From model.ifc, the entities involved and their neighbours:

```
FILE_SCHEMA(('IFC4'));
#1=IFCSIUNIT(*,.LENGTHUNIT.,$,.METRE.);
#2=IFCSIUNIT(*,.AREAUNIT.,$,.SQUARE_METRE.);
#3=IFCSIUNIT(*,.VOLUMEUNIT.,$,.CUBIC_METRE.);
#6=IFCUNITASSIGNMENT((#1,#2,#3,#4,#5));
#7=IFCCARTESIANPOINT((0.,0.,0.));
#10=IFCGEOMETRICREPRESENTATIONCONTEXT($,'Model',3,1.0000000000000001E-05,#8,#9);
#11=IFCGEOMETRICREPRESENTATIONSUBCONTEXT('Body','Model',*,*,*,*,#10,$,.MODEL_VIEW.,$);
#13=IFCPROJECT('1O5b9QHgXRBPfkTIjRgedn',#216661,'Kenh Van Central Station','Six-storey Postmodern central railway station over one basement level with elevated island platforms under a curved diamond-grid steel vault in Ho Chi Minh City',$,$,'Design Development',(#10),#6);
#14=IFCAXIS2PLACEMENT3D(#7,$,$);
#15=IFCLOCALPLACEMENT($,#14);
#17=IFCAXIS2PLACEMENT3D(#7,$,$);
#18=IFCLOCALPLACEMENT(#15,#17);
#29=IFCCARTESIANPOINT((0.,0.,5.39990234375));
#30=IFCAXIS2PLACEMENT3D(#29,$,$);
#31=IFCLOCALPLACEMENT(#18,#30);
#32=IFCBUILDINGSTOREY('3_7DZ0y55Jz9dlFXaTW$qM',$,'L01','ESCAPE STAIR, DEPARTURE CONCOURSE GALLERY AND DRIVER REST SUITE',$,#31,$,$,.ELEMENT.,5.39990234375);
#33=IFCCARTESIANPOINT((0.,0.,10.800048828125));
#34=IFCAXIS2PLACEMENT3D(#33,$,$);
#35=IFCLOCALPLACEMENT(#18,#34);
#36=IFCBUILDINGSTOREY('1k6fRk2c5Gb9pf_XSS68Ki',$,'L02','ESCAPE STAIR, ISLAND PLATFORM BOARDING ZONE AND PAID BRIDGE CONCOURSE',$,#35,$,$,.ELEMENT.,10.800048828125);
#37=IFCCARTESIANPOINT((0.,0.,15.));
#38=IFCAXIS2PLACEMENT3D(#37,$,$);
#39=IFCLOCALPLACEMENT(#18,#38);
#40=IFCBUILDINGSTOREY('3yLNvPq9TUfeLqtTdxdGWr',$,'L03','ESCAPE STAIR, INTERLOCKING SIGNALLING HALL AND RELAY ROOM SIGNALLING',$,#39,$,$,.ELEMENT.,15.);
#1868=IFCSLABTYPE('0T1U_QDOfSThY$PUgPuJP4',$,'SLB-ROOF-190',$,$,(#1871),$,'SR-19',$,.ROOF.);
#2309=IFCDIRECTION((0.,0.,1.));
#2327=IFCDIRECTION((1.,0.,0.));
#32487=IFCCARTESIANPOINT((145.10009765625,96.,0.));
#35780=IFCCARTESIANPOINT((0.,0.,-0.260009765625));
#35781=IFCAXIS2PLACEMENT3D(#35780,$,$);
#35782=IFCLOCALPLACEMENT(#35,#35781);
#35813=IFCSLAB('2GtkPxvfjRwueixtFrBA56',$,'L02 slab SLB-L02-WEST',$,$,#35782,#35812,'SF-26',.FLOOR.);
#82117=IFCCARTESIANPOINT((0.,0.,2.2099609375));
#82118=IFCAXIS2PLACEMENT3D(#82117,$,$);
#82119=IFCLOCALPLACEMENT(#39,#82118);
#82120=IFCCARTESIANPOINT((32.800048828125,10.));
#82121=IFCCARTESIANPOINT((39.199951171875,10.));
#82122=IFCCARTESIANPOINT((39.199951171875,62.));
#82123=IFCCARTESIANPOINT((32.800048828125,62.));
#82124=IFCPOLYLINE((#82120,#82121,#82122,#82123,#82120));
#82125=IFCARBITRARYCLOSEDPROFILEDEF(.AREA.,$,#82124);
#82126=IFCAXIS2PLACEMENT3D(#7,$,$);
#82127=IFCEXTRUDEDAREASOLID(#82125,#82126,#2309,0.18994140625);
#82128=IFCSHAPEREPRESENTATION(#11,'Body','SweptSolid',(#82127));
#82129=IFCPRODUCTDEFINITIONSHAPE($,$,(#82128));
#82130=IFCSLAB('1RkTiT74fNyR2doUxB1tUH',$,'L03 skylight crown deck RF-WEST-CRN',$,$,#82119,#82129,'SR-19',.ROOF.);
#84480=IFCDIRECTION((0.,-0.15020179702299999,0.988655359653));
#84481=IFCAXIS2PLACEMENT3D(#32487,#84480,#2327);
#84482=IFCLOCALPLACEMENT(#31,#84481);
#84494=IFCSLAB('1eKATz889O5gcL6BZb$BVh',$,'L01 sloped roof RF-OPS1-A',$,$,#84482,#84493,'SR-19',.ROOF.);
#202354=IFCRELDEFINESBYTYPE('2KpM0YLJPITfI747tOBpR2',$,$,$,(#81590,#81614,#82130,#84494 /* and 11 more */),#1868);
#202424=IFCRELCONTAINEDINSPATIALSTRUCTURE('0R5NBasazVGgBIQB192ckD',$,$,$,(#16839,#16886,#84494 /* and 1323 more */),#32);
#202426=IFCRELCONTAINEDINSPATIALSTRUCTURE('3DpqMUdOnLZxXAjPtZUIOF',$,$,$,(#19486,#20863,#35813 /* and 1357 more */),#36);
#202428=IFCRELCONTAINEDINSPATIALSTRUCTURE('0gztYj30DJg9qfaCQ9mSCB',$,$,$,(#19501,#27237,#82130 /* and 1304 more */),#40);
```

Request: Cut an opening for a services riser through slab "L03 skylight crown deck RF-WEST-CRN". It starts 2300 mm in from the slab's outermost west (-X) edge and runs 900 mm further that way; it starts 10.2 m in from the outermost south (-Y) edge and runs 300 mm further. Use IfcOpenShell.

```python
import numpy as np
import ifcopenshell
import ifcopenshell.api.feature
import ifcopenshell.api.geometry
import ifcopenshell.api.root
import ifcopenshell.geom
import ifcopenshell.util.placement
import ifcopenshell.util.representation
import ifcopenshell.util.shape
import ifcopenshell.util.unit

model = ifcopenshell.open("model.ifc")
unit_scale = ifcopenshell.util.unit.calculate_unit_scale(model)
settings = ifcopenshell.geom.settings()


def volume(element):
    """Net volume in cubic metres, openings subtracted."""
    shape = ifcopenshell.geom.create_shape(settings, element)
    return ifcopenshell.util.shape.get_volume(shape.geometry)


slab = model.by_guid("1RkTiT74fNyR2doUxB1tUH")
before = volume(slab)

# Extent in the slab's own axes, in metres. The edges named are its -X and -Y sides.
slab_shape = ifcopenshell.geom.create_shape(settings, slab)
vertices = ifcopenshell.util.shape.get_vertices(slab_shape.geometry)
x_min, y_min, bottom = vertices.min(axis=0)
top = vertices[:, 2].max()

opening = ifcopenshell.api.root.create_entity(model, ifc_class="IfcOpeningElement", name="Services riser opening", predefined_type="OPENING")
context = ifcopenshell.util.representation.get_context(model, "Model", "Body", "MODEL_VIEW")
width, depth = 0.9, 0.3
outline = [(0.0, 0.0), (width, 0.0), (width, depth), (0.0, depth), (0.0, 0.0)]
# Overshoot both faces by 50 mm so the cut is clean.
shape = ifcopenshell.api.geometry.add_slab_representation(
    model, context=context, depth=top - bottom + 0.1, polyline=outline
)
ifcopenshell.api.geometry.assign_representation(model, product=opening, representation=shape)

matrix = ifcopenshell.util.placement.get_local_placement(slab.ObjectPlacement)
matrix[:, 3] = matrix @ np.append(np.array([x_min + 2.3, y_min + 10.2, bottom - 0.05]) / unit_scale, 1.0)
ifcopenshell.api.geometry.edit_object_placement(model, product=opening, matrix=matrix, is_si=False)
ifcopenshell.api.feature.add_feature(model, feature=opening, element=slab)

after = volume(slab)

print(f"slab volume {before:.3f} -> {after:.3f} m3")

model.write("model_updated.ifc")
```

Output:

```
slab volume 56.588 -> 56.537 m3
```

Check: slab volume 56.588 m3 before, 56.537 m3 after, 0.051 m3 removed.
